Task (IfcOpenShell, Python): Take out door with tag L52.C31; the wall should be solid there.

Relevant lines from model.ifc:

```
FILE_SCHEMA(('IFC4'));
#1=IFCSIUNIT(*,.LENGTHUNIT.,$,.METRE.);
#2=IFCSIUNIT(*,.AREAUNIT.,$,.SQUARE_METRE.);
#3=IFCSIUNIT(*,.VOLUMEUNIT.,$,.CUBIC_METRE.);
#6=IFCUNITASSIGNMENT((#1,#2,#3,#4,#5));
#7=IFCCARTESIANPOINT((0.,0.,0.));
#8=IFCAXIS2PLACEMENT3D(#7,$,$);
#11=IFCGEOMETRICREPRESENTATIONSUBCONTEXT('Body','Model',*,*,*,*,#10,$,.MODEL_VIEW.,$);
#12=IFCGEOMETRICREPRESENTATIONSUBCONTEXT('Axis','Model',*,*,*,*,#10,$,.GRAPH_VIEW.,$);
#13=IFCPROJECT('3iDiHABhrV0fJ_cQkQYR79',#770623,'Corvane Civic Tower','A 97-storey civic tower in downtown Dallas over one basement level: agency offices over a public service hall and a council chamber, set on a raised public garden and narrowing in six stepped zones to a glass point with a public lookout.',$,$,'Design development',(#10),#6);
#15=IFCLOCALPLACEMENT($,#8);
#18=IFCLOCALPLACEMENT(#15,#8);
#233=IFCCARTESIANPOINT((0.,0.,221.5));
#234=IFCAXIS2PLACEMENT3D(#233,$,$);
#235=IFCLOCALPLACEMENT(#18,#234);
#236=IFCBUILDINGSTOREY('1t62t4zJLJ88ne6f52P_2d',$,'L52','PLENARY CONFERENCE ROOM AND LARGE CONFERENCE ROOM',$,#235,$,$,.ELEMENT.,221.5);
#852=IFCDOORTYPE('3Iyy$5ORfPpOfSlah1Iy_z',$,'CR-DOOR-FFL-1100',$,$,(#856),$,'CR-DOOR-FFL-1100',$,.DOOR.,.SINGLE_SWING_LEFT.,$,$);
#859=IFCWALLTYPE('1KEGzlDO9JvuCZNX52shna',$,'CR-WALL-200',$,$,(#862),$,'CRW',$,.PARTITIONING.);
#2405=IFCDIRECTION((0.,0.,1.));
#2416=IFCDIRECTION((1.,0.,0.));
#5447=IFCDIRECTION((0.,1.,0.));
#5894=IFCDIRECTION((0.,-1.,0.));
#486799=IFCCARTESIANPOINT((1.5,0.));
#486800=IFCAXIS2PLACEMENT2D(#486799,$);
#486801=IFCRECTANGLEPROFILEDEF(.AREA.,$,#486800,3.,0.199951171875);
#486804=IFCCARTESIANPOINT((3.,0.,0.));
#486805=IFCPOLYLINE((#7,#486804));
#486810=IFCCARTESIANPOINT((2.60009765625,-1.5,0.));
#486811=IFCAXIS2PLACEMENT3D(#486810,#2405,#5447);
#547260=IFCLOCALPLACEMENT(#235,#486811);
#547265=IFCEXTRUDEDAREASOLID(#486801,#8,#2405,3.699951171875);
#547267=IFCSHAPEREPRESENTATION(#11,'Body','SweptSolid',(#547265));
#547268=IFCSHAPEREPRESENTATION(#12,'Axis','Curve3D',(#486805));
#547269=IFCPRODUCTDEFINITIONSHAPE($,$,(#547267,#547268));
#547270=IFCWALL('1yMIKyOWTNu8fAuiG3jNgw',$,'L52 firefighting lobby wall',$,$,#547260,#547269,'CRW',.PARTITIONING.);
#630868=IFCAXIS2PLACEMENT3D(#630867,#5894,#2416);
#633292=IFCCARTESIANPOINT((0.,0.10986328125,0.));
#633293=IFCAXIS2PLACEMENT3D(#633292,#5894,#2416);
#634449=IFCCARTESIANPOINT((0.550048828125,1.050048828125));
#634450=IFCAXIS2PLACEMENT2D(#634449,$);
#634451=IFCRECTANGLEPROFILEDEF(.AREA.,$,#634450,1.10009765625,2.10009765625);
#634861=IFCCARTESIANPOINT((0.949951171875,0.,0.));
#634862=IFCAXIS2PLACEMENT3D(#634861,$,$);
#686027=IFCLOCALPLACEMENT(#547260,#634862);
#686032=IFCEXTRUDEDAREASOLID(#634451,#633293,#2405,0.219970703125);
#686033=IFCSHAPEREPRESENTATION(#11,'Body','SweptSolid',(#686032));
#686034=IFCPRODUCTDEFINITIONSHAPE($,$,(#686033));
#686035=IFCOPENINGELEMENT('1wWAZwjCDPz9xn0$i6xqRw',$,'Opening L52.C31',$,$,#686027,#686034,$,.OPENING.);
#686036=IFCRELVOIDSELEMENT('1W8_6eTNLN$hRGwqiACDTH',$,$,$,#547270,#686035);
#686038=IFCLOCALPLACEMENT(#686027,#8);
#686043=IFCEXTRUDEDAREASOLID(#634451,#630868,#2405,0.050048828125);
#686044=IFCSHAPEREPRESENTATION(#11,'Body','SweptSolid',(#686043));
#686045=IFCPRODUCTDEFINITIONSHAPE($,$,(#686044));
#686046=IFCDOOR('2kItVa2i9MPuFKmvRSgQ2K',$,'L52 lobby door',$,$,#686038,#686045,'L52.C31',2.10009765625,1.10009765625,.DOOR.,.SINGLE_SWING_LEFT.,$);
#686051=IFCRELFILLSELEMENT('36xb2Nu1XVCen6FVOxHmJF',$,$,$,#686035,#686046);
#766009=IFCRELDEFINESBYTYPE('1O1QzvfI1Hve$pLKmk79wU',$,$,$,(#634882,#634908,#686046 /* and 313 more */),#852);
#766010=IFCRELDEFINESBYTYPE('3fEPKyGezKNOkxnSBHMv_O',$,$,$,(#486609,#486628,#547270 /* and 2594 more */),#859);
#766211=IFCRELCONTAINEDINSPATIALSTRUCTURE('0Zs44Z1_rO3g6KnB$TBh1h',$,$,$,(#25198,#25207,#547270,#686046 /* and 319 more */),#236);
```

```python
import ifcopenshell
import ifcopenshell.api.feature
import ifcopenshell.api.root
import ifcopenshell.geom
import ifcopenshell.util.shape

model = ifcopenshell.open("model.ifc")
settings = ifcopenshell.geom.settings()


def volume(element):
    """Net volume in cubic metres, openings subtracted."""
    shape = ifcopenshell.geom.create_shape(settings, element)
    return ifcopenshell.util.shape.get_volume(shape.geometry)


door = model.by_id(686046)
opening = door.FillsVoids[0].RelatingOpeningElement
wall = opening.VoidsElements[0].RelatingBuildingElement
before = volume(wall)

ifcopenshell.api.root.remove_product(model, product=door)
ifcopenshell.api.feature.remove_feature(model, feature=opening)

after = volume(wall)

print(f"wall volume {before:.3f} -> {after:.3f} m3")

model.write("model_v2.ifc")
```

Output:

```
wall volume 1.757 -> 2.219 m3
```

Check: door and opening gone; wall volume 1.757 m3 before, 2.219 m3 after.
